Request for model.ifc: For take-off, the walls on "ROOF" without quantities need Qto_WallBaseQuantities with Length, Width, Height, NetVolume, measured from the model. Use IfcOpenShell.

First a look at what the model holds.

```python
import ifcopenshell
import ifcopenshell.util.element
import ifcopenshell.util.unit

model = ifcopenshell.open("model.ifc")
print(model.schema)
for unit_type in ("LENGTHUNIT", "AREAUNIT", "VOLUMEUNIT"):
    print(unit_type, ifcopenshell.util.unit.calculate_unit_scale(model, unit_type))
storey = next(s for s in model.by_type("IfcBuildingStorey") if s.Name == "ROOF")
walls = [e for e in ifcopenshell.util.element.get_decomposition(storey) if e.is_a("IfcWall")]
for e in sorted(walls, key=lambda e: e.id()):
    print(e.id(), e.is_a(), e.Name, list(ifcopenshell.util.element.get_psets(e, qtos_only=True)), sep=" | ")
```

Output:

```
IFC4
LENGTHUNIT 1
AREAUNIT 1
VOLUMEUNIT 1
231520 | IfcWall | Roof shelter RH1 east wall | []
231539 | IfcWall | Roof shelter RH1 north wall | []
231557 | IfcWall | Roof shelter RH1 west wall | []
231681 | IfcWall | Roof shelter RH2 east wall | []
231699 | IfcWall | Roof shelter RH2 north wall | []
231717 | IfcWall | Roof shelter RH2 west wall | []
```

```python
import ifcopenshell
import ifcopenshell.api.pset
import ifcopenshell.geom
import ifcopenshell.util.element
import ifcopenshell.util.shape
import ifcopenshell.util.unit

model = ifcopenshell.open("model.ifc")
unit_scale = ifcopenshell.util.unit.calculate_unit_scale(model)
volume_scale = ifcopenshell.util.unit.calculate_unit_scale(model, "VOLUMEUNIT")
settings = ifcopenshell.geom.settings()

storey = next(s for s in model.by_type("IfcBuildingStorey") if s.Name == "ROOF")
walls = [e for e in ifcopenshell.util.element.get_decomposition(storey) if e.is_a("IfcWall")]

for e in sorted(walls, key=lambda e: e.id()):
    if ifcopenshell.util.element.get_psets(e, qtos_only=True, should_inherit=False):
        continue
    # Geometry comes back in metres, in the element's own axes.
    shape = ifcopenshell.geom.create_shape(settings, e)
    values = {
        "Length": ifcopenshell.util.shape.get_x(shape.geometry) / unit_scale,
        "Width": ifcopenshell.util.shape.get_y(shape.geometry) / unit_scale,
        "Height": ifcopenshell.util.shape.get_z(shape.geometry) / unit_scale,
        "NetVolume": ifcopenshell.util.shape.get_volume(shape.geometry) / volume_scale,
    }
    qto = ifcopenshell.api.pset.add_qto(model, product=e, name="Qto_WallBaseQuantities")
    ifcopenshell.api.pset.edit_qto(model, qto=qto, properties=values)
    print(e.id(), {k: round(v, 3) for k, v in values.items()})

model.write("model_updated.ifc")
```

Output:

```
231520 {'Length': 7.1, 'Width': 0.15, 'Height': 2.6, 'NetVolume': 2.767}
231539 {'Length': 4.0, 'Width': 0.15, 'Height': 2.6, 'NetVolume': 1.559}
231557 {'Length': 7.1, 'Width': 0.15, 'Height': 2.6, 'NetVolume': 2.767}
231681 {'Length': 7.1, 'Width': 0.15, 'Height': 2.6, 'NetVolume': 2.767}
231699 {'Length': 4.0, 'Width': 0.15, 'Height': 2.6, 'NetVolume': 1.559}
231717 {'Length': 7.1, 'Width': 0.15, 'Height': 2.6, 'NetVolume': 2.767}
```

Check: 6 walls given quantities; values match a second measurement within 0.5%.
